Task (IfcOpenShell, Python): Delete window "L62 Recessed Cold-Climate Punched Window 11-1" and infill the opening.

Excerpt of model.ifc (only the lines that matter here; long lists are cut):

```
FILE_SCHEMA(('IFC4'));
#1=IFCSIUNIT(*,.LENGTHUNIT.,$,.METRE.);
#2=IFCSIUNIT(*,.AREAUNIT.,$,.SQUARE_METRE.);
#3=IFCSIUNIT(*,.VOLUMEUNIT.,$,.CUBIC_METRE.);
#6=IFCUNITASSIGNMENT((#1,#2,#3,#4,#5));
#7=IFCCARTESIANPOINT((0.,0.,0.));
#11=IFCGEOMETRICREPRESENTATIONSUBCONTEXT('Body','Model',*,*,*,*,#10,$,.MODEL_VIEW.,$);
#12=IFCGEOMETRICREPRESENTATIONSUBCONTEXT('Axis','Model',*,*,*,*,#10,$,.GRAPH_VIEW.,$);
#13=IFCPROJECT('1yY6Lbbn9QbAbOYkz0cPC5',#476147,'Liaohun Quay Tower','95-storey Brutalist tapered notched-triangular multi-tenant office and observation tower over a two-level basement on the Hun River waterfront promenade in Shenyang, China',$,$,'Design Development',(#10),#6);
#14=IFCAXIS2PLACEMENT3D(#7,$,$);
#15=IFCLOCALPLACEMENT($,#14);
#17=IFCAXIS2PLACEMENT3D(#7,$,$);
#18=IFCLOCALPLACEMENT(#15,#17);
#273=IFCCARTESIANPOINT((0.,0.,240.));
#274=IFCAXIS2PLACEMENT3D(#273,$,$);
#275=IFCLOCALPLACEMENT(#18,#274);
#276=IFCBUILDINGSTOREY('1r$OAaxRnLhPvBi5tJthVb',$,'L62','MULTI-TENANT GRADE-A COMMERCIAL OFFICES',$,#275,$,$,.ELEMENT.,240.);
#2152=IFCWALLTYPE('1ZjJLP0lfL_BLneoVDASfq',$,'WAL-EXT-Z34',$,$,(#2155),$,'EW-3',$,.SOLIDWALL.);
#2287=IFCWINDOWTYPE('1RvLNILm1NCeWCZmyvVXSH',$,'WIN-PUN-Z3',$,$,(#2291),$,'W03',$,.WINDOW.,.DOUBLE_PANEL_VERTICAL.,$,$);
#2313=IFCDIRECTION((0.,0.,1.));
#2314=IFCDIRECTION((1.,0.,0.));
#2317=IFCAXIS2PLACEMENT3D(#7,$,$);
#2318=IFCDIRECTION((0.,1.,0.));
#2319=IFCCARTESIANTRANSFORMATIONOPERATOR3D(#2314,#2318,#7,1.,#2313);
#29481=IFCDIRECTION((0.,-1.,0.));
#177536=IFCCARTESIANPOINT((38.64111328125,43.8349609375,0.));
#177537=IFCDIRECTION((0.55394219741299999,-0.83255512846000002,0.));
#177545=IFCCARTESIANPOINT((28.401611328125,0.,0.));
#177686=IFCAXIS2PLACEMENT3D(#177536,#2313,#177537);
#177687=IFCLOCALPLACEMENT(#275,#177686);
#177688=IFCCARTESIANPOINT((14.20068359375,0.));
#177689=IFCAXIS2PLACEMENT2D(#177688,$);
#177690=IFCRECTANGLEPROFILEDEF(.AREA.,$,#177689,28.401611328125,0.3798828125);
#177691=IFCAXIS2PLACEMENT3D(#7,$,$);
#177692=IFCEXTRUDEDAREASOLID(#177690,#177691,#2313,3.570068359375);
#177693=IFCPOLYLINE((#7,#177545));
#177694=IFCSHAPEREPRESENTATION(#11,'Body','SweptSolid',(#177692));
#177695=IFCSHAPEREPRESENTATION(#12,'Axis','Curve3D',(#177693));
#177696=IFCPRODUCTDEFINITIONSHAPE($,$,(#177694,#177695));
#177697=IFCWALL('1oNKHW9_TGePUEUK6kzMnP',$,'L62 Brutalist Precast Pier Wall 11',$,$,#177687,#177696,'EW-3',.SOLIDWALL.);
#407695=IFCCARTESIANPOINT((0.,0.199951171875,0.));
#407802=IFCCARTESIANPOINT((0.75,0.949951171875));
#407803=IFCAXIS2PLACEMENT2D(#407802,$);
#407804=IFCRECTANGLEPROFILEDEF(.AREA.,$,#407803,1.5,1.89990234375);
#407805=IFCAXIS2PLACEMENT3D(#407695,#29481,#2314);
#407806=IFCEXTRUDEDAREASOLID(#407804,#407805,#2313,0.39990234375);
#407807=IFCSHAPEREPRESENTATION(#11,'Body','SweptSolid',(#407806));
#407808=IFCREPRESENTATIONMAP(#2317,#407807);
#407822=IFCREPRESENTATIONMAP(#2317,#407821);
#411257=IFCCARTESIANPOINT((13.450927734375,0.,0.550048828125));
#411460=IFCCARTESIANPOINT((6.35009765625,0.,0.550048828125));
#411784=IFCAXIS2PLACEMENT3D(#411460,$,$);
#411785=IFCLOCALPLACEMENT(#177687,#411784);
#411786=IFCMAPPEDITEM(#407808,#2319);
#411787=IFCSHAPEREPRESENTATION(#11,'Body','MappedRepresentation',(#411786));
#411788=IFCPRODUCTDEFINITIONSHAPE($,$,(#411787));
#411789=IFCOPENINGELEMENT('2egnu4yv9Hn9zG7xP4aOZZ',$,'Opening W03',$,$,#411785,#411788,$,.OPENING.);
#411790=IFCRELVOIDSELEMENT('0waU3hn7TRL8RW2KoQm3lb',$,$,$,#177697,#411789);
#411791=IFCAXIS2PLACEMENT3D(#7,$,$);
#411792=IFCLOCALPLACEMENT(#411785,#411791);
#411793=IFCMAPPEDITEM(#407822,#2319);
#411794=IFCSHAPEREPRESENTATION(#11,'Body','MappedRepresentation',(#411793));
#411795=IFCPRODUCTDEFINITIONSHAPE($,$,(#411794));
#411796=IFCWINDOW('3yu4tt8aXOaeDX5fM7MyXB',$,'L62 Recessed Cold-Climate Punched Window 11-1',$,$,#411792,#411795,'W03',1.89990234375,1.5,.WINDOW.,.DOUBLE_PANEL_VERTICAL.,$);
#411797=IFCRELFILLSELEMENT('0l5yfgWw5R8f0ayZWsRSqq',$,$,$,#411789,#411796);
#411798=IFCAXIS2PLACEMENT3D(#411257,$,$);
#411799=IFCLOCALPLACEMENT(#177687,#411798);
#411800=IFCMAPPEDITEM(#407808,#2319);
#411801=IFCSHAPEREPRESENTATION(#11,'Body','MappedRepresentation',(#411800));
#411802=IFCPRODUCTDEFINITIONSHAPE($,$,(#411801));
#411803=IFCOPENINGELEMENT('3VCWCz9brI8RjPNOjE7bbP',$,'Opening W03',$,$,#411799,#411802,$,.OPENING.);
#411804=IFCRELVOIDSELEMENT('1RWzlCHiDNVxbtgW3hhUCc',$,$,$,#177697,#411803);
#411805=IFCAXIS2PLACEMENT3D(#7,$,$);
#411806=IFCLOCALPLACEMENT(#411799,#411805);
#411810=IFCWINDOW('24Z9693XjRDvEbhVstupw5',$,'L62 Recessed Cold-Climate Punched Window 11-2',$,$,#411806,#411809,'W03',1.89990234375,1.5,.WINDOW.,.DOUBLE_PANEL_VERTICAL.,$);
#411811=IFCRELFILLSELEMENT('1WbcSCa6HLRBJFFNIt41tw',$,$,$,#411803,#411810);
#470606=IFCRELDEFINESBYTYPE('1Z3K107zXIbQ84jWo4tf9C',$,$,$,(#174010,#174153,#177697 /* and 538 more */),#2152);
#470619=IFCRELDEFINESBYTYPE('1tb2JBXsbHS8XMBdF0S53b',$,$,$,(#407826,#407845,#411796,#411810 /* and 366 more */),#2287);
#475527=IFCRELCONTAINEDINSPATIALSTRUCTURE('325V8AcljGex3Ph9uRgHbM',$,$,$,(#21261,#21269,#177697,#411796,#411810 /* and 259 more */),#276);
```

```python
import ifcopenshell
import ifcopenshell.api.feature
import ifcopenshell.api.root
import ifcopenshell.geom
import ifcopenshell.util.shape

model = ifcopenshell.open("model.ifc")
settings = ifcopenshell.geom.settings()


def volume(element):
    """Net volume in cubic metres, openings subtracted."""
    shape = ifcopenshell.geom.create_shape(settings, element)
    return ifcopenshell.util.shape.get_volume(shape.geometry)


window = model.by_guid("3yu4tt8aXOaeDX5fM7MyXB")
opening = window.FillsVoids[0].RelatingOpeningElement
wall = opening.VoidsElements[0].RelatingBuildingElement
before = volume(wall)

ifcopenshell.api.root.remove_product(model, product=window)
ifcopenshell.api.feature.remove_feature(model, feature=opening)

after = volume(wall)

print(f"wall volume {before:.3f} -> {after:.3f} m3")

model.write("model_updated.ifc")
```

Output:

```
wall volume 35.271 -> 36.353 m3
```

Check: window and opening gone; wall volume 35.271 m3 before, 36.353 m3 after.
